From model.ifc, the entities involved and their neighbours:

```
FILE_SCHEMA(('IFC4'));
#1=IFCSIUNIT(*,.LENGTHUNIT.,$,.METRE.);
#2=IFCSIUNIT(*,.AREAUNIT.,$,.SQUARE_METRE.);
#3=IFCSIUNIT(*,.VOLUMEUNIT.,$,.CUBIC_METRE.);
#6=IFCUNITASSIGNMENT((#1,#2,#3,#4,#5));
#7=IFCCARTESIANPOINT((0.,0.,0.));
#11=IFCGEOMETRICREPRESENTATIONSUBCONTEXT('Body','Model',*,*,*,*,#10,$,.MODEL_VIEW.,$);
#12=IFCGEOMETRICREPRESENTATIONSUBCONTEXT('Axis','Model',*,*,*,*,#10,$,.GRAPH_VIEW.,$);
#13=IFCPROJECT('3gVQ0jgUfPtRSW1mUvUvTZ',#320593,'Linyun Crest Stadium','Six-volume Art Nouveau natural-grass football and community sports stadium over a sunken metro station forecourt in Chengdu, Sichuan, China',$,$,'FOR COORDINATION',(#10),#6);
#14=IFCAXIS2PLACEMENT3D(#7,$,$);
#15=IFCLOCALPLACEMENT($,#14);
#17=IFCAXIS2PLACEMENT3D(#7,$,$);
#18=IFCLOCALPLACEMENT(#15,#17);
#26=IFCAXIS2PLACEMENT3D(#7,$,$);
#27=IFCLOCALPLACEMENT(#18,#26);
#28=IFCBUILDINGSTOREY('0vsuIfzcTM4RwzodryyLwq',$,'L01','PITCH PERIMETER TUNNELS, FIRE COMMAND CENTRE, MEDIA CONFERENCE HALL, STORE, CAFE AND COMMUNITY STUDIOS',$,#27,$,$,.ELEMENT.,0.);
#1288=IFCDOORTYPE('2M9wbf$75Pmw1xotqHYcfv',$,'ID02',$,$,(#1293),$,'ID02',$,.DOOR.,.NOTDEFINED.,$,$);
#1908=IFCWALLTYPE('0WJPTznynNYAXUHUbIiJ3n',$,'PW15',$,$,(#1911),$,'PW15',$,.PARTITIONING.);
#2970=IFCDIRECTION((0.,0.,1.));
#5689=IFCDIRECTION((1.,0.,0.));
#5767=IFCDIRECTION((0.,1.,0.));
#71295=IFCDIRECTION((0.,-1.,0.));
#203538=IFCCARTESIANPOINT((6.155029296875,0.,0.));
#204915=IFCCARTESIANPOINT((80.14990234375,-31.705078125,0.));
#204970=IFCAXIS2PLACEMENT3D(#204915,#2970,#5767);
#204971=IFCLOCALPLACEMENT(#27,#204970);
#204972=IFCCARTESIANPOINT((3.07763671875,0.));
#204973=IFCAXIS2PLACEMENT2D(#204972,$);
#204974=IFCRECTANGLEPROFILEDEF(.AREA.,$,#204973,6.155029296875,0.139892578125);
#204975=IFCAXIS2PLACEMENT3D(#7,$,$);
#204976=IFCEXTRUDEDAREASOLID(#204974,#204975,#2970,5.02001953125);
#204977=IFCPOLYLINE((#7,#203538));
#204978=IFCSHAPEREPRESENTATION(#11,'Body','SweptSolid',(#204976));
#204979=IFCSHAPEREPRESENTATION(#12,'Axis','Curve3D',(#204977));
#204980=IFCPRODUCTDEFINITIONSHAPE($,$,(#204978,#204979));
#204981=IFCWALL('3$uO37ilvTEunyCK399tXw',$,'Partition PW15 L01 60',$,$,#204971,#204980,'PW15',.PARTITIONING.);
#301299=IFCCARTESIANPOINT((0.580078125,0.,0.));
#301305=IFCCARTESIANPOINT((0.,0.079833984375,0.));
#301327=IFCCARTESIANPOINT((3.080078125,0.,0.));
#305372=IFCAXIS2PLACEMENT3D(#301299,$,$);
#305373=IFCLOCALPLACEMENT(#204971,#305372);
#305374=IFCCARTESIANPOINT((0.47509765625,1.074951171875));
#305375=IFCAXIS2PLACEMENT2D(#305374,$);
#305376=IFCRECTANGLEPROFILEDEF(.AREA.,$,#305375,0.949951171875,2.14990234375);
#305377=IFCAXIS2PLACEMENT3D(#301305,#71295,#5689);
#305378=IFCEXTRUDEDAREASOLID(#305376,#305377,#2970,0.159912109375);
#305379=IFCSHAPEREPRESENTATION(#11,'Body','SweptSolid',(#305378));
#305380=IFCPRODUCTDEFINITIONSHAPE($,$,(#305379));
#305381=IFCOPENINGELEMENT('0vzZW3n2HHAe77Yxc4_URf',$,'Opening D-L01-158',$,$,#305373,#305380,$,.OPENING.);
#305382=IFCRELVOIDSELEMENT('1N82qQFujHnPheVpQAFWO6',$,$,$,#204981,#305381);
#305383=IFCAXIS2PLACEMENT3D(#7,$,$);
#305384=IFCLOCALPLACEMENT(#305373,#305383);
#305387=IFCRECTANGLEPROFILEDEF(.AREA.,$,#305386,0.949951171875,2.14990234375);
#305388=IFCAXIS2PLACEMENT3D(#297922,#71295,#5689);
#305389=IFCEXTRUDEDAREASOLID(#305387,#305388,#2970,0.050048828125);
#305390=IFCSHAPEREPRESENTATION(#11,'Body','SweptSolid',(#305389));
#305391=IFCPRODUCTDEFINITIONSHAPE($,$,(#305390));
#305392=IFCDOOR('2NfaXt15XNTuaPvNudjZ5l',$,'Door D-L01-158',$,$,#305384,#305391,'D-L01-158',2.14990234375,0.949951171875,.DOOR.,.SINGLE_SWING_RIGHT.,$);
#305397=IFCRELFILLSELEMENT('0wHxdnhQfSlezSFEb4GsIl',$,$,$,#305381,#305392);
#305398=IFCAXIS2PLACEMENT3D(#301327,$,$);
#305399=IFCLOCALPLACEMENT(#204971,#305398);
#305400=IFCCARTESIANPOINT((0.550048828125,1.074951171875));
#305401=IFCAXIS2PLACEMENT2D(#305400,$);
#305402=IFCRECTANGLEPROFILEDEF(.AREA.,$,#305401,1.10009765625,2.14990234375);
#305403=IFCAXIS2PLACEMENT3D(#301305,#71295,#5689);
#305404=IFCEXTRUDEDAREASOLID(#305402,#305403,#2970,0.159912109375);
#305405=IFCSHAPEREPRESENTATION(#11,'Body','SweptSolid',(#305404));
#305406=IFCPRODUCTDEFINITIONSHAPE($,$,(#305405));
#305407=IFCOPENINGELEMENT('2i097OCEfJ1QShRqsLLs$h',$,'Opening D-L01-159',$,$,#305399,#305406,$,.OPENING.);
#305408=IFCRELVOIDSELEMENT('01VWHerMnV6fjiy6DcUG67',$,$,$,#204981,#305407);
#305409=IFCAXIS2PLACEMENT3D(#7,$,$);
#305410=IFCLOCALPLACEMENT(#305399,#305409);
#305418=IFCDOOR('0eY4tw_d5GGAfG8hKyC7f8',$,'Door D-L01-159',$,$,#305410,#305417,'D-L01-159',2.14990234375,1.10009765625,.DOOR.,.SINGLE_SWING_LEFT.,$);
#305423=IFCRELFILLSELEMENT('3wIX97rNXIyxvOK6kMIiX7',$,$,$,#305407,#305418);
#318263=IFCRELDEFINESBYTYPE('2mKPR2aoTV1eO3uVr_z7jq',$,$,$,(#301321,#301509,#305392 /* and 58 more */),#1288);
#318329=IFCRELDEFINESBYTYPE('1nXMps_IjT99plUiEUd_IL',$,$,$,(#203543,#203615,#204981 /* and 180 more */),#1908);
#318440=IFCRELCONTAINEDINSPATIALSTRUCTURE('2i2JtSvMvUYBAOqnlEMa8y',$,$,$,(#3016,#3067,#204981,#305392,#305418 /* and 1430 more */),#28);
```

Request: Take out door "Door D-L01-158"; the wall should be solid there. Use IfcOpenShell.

```python
import ifcopenshell
import ifcopenshell.api.feature
import ifcopenshell.api.root
import ifcopenshell.geom
import ifcopenshell.util.shape

model = ifcopenshell.open("model.ifc")
settings = ifcopenshell.geom.settings()


def volume(element):
    """Net volume in cubic metres, openings subtracted."""
    shape = ifcopenshell.geom.create_shape(settings, element)
    return ifcopenshell.util.shape.get_volume(shape.geometry)


door = model.by_guid("2NfaXt15XNTuaPvNudjZ5l")
opening = door.FillsVoids[0].RelatingOpeningElement
wall = opening.VoidsElements[0].RelatingBuildingElement
before = volume(wall)

ifcopenshell.api.root.remove_product(model, product=door)
ifcopenshell.api.feature.remove_feature(model, feature=opening)

after = volume(wall)

print(f"wall volume {before:.3f} -> {after:.3f} m3")

model.write("model_edited.ifc")
```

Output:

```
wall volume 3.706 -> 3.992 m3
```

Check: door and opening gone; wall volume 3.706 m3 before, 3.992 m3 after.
